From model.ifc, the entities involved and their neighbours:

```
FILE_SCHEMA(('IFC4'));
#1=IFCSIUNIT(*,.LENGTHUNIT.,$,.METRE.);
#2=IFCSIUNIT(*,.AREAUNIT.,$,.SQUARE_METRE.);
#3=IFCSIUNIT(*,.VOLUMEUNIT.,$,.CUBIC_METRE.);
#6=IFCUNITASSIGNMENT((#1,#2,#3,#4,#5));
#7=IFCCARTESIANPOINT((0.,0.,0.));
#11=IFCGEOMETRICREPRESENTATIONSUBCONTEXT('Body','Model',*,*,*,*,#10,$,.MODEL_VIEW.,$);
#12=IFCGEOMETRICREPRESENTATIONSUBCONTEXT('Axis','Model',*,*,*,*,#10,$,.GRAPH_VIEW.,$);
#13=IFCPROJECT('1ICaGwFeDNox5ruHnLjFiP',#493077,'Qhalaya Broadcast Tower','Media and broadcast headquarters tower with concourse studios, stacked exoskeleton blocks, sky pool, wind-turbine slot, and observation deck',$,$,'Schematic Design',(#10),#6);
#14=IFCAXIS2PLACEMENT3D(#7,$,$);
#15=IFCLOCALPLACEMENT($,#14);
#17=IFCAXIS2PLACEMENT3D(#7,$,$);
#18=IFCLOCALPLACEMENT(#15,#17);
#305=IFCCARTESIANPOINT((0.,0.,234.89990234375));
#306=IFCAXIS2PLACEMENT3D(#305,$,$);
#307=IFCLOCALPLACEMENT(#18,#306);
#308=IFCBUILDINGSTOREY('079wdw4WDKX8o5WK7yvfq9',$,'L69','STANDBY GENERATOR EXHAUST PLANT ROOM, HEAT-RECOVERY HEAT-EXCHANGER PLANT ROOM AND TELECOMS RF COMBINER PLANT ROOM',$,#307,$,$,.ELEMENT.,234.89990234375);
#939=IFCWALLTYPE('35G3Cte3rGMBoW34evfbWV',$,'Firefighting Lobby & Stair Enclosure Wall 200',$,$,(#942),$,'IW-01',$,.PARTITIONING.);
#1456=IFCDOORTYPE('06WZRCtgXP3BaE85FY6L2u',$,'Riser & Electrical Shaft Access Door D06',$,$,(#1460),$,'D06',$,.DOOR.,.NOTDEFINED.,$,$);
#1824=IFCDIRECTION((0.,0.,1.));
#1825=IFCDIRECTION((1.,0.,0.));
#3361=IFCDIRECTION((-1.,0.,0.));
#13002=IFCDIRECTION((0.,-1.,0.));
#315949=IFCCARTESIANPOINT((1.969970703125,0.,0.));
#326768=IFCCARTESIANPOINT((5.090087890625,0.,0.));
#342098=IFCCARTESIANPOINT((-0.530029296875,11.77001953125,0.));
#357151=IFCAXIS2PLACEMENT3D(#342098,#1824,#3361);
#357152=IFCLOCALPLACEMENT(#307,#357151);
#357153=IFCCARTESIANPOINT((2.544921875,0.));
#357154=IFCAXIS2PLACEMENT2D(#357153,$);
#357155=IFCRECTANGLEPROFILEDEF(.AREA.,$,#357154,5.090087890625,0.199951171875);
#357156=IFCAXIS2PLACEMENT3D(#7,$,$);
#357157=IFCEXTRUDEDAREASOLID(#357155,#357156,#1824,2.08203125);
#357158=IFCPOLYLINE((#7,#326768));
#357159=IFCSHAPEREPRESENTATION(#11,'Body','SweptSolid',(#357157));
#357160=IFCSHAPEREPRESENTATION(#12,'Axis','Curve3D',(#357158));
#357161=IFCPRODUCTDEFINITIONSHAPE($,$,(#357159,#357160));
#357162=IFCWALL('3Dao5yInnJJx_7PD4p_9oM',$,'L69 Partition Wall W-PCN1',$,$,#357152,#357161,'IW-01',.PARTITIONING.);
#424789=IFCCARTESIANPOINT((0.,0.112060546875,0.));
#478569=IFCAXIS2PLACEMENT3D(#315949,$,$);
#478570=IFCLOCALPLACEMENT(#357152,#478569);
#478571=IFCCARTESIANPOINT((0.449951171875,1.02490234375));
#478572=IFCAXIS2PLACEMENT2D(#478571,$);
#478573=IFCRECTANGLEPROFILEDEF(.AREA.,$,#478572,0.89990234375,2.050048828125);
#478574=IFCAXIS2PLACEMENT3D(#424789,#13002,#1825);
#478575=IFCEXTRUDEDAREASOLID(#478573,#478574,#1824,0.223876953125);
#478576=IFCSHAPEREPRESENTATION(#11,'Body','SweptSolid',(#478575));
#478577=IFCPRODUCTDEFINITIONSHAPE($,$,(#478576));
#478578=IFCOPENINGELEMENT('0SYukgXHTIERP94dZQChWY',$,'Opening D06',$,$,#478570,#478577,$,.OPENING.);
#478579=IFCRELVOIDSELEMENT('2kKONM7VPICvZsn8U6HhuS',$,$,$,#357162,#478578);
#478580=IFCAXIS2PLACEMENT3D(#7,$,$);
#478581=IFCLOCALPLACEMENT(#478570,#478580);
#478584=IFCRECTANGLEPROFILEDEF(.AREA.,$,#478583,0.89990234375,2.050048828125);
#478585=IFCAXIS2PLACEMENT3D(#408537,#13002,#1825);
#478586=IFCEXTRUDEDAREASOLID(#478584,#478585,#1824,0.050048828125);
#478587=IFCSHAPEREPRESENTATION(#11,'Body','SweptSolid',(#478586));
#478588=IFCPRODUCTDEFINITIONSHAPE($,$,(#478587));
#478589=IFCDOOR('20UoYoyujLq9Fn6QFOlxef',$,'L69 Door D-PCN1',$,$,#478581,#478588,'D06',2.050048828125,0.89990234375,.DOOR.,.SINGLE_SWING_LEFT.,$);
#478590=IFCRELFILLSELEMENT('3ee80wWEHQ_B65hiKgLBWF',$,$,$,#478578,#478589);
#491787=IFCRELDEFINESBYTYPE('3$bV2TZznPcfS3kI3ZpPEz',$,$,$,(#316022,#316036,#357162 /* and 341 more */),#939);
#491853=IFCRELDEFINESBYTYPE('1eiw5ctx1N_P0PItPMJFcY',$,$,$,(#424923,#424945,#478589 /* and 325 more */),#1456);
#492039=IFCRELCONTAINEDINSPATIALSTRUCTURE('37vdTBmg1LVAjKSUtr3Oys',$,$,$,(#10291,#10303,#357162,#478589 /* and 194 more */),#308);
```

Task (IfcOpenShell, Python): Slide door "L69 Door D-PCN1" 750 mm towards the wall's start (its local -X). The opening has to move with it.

```python
import ifcopenshell
import ifcopenshell.api.geometry
import ifcopenshell.util.placement
import ifcopenshell.util.unit

model = ifcopenshell.open("model.ifc")
unit_scale = ifcopenshell.util.unit.calculate_unit_scale(model)

door = model.by_guid("20UoYoyujLq9Fn6QFOlxef")
opening = door.FillsVoids[0].RelatingOpeningElement
wall = opening.VoidsElements[0].RelatingBuildingElement

wall_matrix = ifcopenshell.util.placement.get_local_placement(wall.ObjectPlacement)
shift = wall_matrix[:3, 0] * -0.75 / unit_scale
before = ifcopenshell.util.placement.get_local_placement(door.ObjectPlacement)[:3, 3].copy()

# The door is placed relative to its opening, so it follows when the opening moves.
matrix = ifcopenshell.util.placement.get_local_placement(opening.ObjectPlacement)
matrix[:3, 3] += shift
ifcopenshell.api.geometry.edit_object_placement(
    model, product=opening, matrix=matrix, is_si=False, should_transform_children=True
)

after = ifcopenshell.util.placement.get_local_placement(door.ObjectPlacement)[:3, 3]
print("door moved by", (after - before).round(3) + 0.0)

model.write("model-out.ifc")
```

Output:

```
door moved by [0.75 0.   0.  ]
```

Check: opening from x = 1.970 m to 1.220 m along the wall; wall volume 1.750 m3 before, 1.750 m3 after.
